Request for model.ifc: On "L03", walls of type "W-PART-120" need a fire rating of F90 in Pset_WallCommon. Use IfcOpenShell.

First a look at what the model holds.

```python
import ifcopenshell
import ifcopenshell.util.element

model = ifcopenshell.open("model.ifc")
print(model.schema)
storey = next(s for s in model.by_type("IfcBuildingStorey") if s.Name == "L03")
walls = [e for e in ifcopenshell.util.element.get_decomposition(storey) if e.is_a("IfcWall")]
seen = {}
for e in walls:
    element_type = ifcopenshell.util.element.get_type(e)
    key = (element_type.Name if element_type != e and element_type else None, ifcopenshell.util.element.get_pset(e, "Pset_WallCommon", "FireRating"))
    seen[key] = seen.get(key, 0) + 1
for (name, value), count in sorted(seen.items(), key=str):
    print(count, "x", name, "|", value)
```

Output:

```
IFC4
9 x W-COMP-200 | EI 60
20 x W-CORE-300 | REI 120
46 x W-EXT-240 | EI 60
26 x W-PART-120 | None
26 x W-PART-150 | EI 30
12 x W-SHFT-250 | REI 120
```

```python
import ifcopenshell
import ifcopenshell.api.pset
import ifcopenshell.util.element

model = ifcopenshell.open("model.ifc")

storey = next(s for s in model.by_type("IfcBuildingStorey") if s.Name == "L03")
walls = [e for e in ifcopenshell.util.element.get_decomposition(storey) if e.is_a("IfcWall")]

count = 0
for e in walls:
    element_type = ifcopenshell.util.element.get_type(e)
    if element_type in (None, e) or element_type.Name != "W-PART-120":
        continue
    # add_pset returns the element's existing set when there is one.
    pset = ifcopenshell.api.pset.add_pset(model, product=e, name="Pset_WallCommon")
    ifcopenshell.api.pset.edit_pset(model, pset=pset, properties={"FireRating": "F90"})
    count += 1

print(count, "walls updated")

model.write("model_edited.ifc")
```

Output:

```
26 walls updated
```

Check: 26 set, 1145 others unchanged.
